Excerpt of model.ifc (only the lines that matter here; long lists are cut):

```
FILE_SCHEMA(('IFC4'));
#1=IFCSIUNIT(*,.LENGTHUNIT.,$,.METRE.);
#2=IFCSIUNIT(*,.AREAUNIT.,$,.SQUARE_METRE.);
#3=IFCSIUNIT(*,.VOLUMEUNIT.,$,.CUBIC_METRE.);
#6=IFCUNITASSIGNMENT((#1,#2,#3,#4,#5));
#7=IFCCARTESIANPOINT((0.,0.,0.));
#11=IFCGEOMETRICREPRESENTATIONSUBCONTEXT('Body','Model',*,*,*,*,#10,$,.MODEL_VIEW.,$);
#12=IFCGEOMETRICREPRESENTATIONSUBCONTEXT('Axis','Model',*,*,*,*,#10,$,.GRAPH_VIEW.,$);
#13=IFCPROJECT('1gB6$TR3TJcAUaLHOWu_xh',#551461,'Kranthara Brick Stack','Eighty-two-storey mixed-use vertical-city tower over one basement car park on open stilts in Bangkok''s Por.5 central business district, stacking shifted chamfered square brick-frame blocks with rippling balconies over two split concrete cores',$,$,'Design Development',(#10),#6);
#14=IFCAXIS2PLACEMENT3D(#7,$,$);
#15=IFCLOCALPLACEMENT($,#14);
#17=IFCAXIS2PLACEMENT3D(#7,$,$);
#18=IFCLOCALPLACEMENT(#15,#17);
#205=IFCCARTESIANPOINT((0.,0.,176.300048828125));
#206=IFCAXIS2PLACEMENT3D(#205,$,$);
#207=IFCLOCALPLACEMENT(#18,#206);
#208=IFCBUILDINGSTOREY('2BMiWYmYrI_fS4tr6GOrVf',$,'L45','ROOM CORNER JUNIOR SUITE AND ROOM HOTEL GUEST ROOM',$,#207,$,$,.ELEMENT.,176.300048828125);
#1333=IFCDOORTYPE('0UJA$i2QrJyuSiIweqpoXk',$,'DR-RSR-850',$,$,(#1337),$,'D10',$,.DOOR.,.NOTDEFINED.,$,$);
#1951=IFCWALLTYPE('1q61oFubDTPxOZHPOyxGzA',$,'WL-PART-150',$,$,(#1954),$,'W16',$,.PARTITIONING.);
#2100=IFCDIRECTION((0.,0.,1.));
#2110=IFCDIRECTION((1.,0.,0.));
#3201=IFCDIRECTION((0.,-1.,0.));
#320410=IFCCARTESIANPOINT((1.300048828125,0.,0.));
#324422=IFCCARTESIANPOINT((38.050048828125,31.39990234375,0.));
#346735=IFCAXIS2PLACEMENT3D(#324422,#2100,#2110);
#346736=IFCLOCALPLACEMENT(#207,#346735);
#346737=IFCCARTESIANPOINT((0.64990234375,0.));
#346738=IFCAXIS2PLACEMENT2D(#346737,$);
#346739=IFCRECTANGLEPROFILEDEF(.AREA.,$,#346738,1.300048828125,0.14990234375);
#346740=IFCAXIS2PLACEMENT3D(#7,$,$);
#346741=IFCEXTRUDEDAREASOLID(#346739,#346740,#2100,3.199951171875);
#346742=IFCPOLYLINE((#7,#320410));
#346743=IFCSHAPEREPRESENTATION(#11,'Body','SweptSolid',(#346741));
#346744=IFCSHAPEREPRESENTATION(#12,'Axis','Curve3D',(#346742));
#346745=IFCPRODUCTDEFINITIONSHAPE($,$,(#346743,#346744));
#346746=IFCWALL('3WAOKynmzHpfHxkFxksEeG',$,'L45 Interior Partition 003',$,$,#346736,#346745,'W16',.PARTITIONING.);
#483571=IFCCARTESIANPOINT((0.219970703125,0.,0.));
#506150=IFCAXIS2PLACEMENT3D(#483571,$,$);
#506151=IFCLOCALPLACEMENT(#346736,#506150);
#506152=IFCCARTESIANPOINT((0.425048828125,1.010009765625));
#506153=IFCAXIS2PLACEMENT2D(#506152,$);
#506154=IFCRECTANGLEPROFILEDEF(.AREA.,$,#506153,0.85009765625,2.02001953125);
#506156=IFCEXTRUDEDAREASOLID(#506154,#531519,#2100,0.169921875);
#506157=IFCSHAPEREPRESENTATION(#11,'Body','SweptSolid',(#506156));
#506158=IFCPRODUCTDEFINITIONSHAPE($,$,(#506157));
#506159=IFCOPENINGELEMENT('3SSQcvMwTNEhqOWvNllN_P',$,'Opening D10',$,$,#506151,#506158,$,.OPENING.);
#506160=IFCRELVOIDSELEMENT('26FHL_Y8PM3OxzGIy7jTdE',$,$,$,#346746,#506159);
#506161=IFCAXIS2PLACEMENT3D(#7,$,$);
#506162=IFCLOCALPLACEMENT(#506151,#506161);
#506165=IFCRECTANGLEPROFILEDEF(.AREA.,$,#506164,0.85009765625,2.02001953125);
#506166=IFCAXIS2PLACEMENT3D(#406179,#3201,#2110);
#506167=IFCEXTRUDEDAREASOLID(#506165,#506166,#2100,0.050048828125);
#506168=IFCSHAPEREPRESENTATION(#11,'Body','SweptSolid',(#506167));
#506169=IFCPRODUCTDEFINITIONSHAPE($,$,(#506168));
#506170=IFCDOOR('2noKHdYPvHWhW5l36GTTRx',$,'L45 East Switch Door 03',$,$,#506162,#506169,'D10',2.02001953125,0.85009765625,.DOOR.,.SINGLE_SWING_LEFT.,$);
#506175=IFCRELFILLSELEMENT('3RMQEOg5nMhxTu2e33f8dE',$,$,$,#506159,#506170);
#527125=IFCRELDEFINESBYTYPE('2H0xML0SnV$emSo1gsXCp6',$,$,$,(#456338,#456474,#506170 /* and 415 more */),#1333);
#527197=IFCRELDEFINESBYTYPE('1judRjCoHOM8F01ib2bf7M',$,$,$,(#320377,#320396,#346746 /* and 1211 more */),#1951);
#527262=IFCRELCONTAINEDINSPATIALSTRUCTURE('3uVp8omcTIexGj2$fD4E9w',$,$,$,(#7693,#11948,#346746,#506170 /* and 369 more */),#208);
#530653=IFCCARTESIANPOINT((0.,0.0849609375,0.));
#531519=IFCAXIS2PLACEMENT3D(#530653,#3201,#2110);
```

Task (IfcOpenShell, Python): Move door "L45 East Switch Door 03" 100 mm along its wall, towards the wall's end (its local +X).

```python
import ifcopenshell
import ifcopenshell.api.geometry
import ifcopenshell.util.placement
import ifcopenshell.util.unit

model = ifcopenshell.open("model.ifc")
unit_scale = ifcopenshell.util.unit.calculate_unit_scale(model)

door = model.by_guid("2noKHdYPvHWhW5l36GTTRx")
opening = door.FillsVoids[0].RelatingOpeningElement
wall = opening.VoidsElements[0].RelatingBuildingElement

wall_matrix = ifcopenshell.util.placement.get_local_placement(wall.ObjectPlacement)
shift = wall_matrix[:3, 0] * 0.1 / unit_scale
before = ifcopenshell.util.placement.get_local_placement(door.ObjectPlacement)[:3, 3].copy()

# The door is placed relative to its opening, so it follows when the opening moves.
matrix = ifcopenshell.util.placement.get_local_placement(opening.ObjectPlacement)
matrix[:3, 3] += shift
ifcopenshell.api.geometry.edit_object_placement(
    model, product=opening, matrix=matrix, is_si=False, should_transform_children=True
)

after = ifcopenshell.util.placement.get_local_placement(door.ObjectPlacement)[:3, 3]
print("door moved by", (after - before).round(3) + 0.0)

model.write("model_rev.ifc")
```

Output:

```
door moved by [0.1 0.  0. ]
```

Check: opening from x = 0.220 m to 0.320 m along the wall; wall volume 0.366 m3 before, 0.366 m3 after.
